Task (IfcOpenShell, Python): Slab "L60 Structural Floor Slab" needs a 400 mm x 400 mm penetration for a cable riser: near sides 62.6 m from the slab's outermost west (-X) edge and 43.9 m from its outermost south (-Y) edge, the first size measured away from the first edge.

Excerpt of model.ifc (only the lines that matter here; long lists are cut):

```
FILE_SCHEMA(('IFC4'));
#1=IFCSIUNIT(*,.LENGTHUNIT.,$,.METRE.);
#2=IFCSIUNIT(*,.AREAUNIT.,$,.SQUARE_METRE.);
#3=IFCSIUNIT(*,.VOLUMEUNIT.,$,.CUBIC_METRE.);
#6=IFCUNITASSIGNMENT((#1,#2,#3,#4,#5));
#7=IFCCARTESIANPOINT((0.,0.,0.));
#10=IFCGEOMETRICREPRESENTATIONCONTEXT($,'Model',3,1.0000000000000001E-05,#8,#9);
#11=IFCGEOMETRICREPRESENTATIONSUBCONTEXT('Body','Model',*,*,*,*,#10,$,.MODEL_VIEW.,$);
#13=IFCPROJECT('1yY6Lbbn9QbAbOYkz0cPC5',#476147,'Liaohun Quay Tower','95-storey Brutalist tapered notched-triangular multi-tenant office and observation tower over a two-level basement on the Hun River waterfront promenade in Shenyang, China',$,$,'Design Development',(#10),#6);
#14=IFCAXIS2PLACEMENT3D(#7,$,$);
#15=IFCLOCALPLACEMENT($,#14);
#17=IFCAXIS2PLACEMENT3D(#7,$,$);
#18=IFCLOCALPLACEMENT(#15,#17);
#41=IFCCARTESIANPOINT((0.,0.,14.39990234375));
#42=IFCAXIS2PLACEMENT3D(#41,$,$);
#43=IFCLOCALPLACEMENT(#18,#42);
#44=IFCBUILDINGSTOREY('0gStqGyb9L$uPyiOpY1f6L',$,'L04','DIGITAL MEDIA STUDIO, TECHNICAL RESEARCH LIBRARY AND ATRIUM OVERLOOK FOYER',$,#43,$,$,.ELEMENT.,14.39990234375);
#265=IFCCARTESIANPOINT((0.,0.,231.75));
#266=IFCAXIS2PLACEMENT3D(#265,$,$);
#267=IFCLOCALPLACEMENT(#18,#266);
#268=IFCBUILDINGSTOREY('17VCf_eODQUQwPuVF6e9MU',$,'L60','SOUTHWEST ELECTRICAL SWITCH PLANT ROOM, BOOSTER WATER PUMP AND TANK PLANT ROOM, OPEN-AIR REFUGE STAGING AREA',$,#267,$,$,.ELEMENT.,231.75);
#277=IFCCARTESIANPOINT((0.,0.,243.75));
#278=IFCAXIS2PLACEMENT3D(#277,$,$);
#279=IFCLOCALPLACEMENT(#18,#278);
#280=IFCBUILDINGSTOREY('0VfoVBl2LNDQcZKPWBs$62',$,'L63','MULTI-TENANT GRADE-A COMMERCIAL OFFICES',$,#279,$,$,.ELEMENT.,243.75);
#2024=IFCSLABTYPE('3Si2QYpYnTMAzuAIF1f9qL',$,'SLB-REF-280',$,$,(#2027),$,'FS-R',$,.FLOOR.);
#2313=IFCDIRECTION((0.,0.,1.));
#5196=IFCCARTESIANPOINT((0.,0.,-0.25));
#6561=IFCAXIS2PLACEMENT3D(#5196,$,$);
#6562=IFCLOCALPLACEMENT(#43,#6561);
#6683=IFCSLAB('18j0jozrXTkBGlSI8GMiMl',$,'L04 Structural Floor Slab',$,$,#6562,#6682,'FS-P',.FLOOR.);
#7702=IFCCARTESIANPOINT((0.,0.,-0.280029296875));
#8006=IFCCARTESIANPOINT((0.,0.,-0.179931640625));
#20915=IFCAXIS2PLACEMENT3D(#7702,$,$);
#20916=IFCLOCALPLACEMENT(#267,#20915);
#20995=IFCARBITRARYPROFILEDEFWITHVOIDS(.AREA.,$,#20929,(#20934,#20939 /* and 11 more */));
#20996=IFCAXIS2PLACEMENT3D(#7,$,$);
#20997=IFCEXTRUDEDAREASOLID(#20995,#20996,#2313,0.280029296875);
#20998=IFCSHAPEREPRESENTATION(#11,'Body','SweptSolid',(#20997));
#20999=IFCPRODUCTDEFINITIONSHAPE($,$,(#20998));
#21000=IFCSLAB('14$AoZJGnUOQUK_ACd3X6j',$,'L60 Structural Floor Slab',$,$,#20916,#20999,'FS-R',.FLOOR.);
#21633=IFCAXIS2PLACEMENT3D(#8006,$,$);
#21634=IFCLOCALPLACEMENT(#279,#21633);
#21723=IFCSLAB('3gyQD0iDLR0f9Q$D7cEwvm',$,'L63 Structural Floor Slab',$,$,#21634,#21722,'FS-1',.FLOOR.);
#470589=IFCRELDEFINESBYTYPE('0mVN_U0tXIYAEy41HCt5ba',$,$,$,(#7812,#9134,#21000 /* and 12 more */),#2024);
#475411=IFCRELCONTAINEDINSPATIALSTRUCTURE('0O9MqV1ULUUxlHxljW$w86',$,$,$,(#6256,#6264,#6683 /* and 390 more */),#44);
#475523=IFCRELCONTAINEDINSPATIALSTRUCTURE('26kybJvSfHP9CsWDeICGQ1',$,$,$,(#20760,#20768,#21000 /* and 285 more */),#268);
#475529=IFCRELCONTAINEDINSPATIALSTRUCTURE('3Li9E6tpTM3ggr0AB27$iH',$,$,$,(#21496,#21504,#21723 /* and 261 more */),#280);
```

```python
import numpy as np
import ifcopenshell
import ifcopenshell.api.feature
import ifcopenshell.api.geometry
import ifcopenshell.api.root
import ifcopenshell.geom
import ifcopenshell.util.placement
import ifcopenshell.util.representation
import ifcopenshell.util.shape
import ifcopenshell.util.unit

model = ifcopenshell.open("model.ifc")
unit_scale = ifcopenshell.util.unit.calculate_unit_scale(model)
settings = ifcopenshell.geom.settings()


def volume(element):
    """Net volume in cubic metres, openings subtracted."""
    shape = ifcopenshell.geom.create_shape(settings, element)
    return ifcopenshell.util.shape.get_volume(shape.geometry)


slab = model.by_guid("14$AoZJGnUOQUK_ACd3X6j")
before = volume(slab)

# Extent in the slab's own axes, in metres. The edges named are its -X and -Y sides.
slab_shape = ifcopenshell.geom.create_shape(settings, slab)
vertices = ifcopenshell.util.shape.get_vertices(slab_shape.geometry)
x_min, y_min, bottom = vertices.min(axis=0)
top = vertices[:, 2].max()

opening = ifcopenshell.api.root.create_entity(model, ifc_class="IfcOpeningElement", name="Cable riser opening", predefined_type="OPENING")
context = ifcopenshell.util.representation.get_context(model, "Model", "Body", "MODEL_VIEW")
width, depth = 0.4, 0.4
outline = [(0.0, 0.0), (width, 0.0), (width, depth), (0.0, depth), (0.0, 0.0)]
# Overshoot both faces by 50 mm so the cut is clean.
shape = ifcopenshell.api.geometry.add_slab_representation(
    model, context=context, depth=top - bottom + 0.1, polyline=outline
)
ifcopenshell.api.geometry.assign_representation(model, product=opening, representation=shape)

matrix = ifcopenshell.util.placement.get_local_placement(slab.ObjectPlacement)
matrix[:, 3] = matrix @ np.append(np.array([x_min + 62.6, y_min + 43.9, bottom - 0.05]) / unit_scale, 1.0)
ifcopenshell.api.geometry.edit_object_placement(model, product=opening, matrix=matrix, is_si=False)
ifcopenshell.api.feature.add_feature(model, feature=opening, element=slab)

after = volume(slab)

print(f"slab volume {before:.3f} -> {after:.3f} m3")

model.write("model_rev.ifc")
```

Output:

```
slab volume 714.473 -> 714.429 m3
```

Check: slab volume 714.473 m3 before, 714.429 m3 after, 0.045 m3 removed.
